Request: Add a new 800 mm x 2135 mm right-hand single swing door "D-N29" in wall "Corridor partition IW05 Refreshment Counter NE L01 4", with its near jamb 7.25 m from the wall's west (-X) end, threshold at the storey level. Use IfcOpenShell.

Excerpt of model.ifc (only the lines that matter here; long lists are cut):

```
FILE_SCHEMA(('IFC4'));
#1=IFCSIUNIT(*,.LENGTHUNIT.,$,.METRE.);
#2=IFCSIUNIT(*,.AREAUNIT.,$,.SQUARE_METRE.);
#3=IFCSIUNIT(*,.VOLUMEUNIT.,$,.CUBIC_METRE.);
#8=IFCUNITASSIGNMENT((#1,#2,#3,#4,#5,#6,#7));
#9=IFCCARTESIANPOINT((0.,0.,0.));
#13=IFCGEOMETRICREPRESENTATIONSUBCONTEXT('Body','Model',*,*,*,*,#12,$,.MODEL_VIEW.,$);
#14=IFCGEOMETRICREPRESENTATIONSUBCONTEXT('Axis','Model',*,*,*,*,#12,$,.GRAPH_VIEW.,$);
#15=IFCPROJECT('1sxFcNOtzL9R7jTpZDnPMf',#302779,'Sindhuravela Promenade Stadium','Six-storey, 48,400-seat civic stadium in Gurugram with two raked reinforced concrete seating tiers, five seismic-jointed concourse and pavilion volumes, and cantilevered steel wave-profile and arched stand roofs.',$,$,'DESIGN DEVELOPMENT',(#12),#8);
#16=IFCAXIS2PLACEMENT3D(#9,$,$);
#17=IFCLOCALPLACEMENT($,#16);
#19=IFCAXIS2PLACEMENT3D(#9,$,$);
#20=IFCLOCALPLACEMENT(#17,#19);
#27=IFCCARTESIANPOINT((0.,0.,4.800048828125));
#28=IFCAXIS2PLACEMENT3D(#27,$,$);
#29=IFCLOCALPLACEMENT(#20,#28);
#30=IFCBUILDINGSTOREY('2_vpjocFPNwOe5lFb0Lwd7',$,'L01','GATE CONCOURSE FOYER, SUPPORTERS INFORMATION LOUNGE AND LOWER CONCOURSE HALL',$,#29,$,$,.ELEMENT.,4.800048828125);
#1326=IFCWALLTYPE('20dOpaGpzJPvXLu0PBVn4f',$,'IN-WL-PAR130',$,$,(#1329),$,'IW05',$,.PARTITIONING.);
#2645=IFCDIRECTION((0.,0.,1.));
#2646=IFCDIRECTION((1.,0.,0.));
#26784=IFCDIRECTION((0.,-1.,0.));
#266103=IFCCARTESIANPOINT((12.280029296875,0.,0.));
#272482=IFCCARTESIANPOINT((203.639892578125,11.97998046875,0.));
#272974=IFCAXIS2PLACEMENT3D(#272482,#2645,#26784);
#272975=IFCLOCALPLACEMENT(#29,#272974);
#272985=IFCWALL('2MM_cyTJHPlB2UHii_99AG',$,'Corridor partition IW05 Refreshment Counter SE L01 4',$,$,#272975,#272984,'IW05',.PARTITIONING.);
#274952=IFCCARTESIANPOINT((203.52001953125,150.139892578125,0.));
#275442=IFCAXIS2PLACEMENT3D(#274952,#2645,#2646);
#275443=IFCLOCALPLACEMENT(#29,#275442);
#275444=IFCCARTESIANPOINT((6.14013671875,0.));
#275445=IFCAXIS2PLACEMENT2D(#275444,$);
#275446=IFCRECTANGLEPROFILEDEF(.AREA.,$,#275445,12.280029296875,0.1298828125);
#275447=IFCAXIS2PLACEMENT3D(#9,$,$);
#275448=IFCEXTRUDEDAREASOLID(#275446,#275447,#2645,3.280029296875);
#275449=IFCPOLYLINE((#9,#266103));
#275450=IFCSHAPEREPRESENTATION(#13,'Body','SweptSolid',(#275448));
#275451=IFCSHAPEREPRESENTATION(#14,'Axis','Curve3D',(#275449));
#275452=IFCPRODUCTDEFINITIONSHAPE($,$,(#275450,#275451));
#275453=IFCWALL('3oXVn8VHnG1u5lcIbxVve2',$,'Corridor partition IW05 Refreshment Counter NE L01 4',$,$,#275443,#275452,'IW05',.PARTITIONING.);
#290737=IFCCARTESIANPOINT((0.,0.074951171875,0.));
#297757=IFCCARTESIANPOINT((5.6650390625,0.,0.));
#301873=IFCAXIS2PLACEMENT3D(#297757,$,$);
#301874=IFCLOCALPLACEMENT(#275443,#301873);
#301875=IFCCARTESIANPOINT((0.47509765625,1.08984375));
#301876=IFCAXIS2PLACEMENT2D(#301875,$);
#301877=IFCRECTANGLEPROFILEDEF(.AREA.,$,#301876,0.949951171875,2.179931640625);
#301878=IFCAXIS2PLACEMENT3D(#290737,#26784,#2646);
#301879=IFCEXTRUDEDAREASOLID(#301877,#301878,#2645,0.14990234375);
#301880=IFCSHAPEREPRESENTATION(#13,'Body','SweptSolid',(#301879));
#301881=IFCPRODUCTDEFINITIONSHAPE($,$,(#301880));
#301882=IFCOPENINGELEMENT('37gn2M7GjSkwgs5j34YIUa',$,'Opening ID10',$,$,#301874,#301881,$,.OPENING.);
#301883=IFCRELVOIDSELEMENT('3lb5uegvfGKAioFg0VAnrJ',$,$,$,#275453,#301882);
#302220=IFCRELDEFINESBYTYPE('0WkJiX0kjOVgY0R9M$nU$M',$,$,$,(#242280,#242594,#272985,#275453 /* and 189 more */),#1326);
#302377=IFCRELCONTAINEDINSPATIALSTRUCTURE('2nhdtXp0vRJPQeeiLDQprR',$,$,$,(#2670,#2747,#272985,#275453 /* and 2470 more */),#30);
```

```python
import numpy as np
import ifcopenshell
import ifcopenshell.api.feature
import ifcopenshell.api.geometry
import ifcopenshell.api.root
import ifcopenshell.api.spatial
import ifcopenshell.geom
import ifcopenshell.util.element
import ifcopenshell.util.placement
import ifcopenshell.util.representation
import ifcopenshell.util.shape
import ifcopenshell.util.unit

model = ifcopenshell.open("model.ifc")
unit_scale = ifcopenshell.util.unit.calculate_unit_scale(model)
settings = ifcopenshell.geom.settings()


def volume(element):
    """Net volume in cubic metres, openings subtracted."""
    shape = ifcopenshell.geom.create_shape(settings, element)
    return ifcopenshell.util.shape.get_volume(shape.geometry)


wall = model.by_id(275453)
storey = ifcopenshell.util.element.get_container(wall, ifc_class="IfcBuildingStorey")
context = ifcopenshell.util.representation.get_context(model, "Model", "Body", "MODEL_VIEW")
before = volume(wall)

width, height, from_end, sill = 0.8, 2.135, 7.25, 0.0  # metres

# The wall runs along its own X axis, and the end named is its -X end.
wall_shape = ifcopenshell.geom.create_shape(settings, wall)
x, y, z = ifcopenshell.util.shape.get_vertices(wall_shape.geometry).T
start = x.min() + from_end
face, thickness = float(y.min()), float(y.max() - y.min())
wall_matrix = ifcopenshell.util.placement.get_local_placement(wall.ObjectPlacement)
level = ifcopenshell.util.placement.get_local_placement(storey.ObjectPlacement)[2, 3]


def in_wall(x, y):
    """Placement at x, y metres in the wall's axes, at sill height."""
    matrix = wall_matrix.copy()
    matrix[:, 3] = wall_matrix @ np.array([x / unit_scale, y / unit_scale, 0.0, 1.0])
    matrix[2, 3] = level + sill / unit_scale
    return matrix


# Opening: a box that overshoots both wall faces by 50 mm.
opening = ifcopenshell.api.root.create_entity(model, ifc_class="IfcOpeningElement", predefined_type="OPENING")
box = ifcopenshell.api.geometry.add_wall_representation(
    model, context=context, length=width, height=height, thickness=thickness + 0.1
)
ifcopenshell.api.geometry.assign_representation(model, product=opening, representation=box)
ifcopenshell.api.geometry.edit_object_placement(model, product=opening, matrix=in_wall(start, face - 0.05), is_si=False)
ifcopenshell.api.feature.add_feature(model, feature=opening, element=wall)

door = ifcopenshell.api.root.create_entity(model, ifc_class="IfcDoor", name="D-N29", predefined_type="DOOR")
door.OverallWidth, door.OverallHeight = width / unit_scale, height / unit_scale
door.OperationType = "SINGLE_SWING_RIGHT"
body = ifcopenshell.api.geometry.add_door_representation(
    model,
    context=context,
    overall_width=door.OverallWidth,
    overall_height=door.OverallHeight,
    operation_type="SINGLE_SWING_RIGHT",
    lining_properties={"LiningDepth": thickness / unit_scale, "ThresholdDepth": thickness / unit_scale},
)
ifcopenshell.api.geometry.assign_representation(model, product=door, representation=body)
ifcopenshell.api.spatial.assign_container(model, products=[door], relating_structure=storey)
ifcopenshell.api.feature.add_filling(model, opening=opening, element=door)

# The lining spans the wall, so the door starts at the wall face.
ifcopenshell.api.geometry.edit_object_placement(model, product=door, matrix=in_wall(start, face), is_si=False)

after = volume(wall)

print(f"wall volume {before:.3f} -> {after:.3f} m3")

model.write("model-out.ifc")
```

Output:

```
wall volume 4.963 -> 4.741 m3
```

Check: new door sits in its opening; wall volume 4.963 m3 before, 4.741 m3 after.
